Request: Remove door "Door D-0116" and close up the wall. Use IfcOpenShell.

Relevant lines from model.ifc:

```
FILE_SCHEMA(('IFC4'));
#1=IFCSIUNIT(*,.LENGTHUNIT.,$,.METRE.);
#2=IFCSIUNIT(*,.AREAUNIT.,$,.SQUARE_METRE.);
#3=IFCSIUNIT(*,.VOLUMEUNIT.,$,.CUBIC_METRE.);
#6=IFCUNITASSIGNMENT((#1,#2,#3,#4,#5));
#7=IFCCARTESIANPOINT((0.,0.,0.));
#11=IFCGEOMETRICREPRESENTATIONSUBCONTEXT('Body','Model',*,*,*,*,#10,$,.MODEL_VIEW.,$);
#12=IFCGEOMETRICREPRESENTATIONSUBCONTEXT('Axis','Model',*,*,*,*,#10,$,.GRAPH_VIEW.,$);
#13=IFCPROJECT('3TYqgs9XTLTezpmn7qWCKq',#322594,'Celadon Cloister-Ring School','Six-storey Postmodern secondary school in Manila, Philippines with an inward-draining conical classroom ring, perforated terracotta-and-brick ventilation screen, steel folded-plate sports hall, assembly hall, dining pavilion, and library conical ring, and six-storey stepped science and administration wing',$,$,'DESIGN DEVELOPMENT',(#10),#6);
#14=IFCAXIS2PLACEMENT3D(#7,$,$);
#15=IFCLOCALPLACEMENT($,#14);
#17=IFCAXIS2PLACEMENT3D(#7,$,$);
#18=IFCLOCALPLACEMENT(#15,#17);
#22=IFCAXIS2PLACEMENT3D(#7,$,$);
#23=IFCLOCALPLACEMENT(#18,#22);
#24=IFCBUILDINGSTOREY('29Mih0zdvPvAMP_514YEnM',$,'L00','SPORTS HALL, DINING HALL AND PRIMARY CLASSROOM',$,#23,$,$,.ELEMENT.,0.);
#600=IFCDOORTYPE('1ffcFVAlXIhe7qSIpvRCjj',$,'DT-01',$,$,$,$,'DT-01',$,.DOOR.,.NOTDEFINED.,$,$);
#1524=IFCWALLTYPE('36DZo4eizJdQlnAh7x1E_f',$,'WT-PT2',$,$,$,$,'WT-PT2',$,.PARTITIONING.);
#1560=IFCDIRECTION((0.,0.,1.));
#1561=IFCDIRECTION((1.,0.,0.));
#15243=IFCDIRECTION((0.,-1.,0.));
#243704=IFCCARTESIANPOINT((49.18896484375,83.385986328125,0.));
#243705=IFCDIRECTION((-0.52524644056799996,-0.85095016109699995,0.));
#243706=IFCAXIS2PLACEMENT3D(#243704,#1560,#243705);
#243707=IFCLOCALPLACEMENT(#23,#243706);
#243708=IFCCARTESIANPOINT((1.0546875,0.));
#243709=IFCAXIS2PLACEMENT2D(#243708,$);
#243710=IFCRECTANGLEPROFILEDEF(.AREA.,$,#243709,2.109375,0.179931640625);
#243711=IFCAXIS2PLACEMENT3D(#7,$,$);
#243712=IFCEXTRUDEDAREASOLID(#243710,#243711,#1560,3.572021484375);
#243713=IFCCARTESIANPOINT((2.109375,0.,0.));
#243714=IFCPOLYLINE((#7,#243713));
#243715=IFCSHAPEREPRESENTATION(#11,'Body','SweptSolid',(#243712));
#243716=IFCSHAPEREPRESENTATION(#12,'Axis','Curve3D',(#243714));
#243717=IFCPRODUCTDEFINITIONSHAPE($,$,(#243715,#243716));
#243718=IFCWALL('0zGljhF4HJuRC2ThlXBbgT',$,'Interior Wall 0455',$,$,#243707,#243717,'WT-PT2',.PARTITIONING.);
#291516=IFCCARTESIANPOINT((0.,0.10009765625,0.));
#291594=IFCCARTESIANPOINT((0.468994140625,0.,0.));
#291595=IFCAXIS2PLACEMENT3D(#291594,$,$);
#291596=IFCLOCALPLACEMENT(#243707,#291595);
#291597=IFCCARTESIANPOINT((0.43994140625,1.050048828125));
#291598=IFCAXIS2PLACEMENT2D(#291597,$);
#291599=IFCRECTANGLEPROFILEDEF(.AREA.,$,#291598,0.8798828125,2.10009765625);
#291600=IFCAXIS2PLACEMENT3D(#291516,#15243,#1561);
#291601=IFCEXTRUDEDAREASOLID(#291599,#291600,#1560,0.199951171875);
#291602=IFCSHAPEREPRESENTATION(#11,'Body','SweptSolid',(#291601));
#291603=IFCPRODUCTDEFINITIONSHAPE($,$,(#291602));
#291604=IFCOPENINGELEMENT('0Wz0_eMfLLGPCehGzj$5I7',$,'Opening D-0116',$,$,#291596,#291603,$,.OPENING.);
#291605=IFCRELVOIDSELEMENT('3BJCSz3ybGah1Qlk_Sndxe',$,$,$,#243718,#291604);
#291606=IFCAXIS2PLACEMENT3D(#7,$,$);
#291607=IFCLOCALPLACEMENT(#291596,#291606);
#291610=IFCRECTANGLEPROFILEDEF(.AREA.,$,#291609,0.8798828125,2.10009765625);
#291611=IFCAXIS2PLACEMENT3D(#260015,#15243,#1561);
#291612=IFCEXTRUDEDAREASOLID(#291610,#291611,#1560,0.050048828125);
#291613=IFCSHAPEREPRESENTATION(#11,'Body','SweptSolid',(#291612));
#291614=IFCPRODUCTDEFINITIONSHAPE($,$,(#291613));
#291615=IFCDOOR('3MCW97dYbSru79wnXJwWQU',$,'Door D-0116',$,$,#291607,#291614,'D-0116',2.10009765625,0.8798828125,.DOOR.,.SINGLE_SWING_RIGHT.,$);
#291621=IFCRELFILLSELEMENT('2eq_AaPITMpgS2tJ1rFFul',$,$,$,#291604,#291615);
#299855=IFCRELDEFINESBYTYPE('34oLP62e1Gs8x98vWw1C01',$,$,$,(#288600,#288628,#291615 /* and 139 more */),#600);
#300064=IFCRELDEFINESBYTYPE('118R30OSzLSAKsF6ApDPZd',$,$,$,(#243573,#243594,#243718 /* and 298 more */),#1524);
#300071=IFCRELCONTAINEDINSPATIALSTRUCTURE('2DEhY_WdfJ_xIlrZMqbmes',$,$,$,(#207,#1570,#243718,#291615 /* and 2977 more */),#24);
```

```python
import ifcopenshell
import ifcopenshell.api.feature
import ifcopenshell.api.root
import ifcopenshell.geom
import ifcopenshell.util.shape

model = ifcopenshell.open("model.ifc")
settings = ifcopenshell.geom.settings()


def volume(element):
    """Net volume in cubic metres, openings subtracted."""
    shape = ifcopenshell.geom.create_shape(settings, element)
    return ifcopenshell.util.shape.get_volume(shape.geometry)


door = model.by_guid("3MCW97dYbSru79wnXJwWQU")
opening = door.FillsVoids[0].RelatingOpeningElement
wall = opening.VoidsElements[0].RelatingBuildingElement
before = volume(wall)

ifcopenshell.api.root.remove_product(model, product=door)
ifcopenshell.api.feature.remove_feature(model, feature=opening)

after = volume(wall)

print(f"wall volume {before:.3f} -> {after:.3f} m3")

model.write("model-out.ifc")
```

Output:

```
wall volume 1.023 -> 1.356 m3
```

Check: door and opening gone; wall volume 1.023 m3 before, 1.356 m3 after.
